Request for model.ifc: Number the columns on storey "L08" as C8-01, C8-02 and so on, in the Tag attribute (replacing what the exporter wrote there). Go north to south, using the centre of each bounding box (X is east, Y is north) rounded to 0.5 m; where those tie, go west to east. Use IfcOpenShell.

First a look at what the model holds.

```python
import ifcopenshell
import ifcopenshell.util.element
import ifcopenshell.util.placement

model = ifcopenshell.open("model.ifc")
print(model.schema)
storey = next(s for s in model.by_type("IfcBuildingStorey") if s.Name == "L08")
columns = [e for e in ifcopenshell.util.element.get_decomposition(storey) if e.is_a("IfcColumn")]
for e in sorted(columns, key=lambda e: e.id()):
    origin = ifcopenshell.util.placement.get_local_placement(e.ObjectPlacement)[:3, 3]
    print(e.id(), e.Tag, e.Name, origin.round(2) + 0.0, sep=" | ")
```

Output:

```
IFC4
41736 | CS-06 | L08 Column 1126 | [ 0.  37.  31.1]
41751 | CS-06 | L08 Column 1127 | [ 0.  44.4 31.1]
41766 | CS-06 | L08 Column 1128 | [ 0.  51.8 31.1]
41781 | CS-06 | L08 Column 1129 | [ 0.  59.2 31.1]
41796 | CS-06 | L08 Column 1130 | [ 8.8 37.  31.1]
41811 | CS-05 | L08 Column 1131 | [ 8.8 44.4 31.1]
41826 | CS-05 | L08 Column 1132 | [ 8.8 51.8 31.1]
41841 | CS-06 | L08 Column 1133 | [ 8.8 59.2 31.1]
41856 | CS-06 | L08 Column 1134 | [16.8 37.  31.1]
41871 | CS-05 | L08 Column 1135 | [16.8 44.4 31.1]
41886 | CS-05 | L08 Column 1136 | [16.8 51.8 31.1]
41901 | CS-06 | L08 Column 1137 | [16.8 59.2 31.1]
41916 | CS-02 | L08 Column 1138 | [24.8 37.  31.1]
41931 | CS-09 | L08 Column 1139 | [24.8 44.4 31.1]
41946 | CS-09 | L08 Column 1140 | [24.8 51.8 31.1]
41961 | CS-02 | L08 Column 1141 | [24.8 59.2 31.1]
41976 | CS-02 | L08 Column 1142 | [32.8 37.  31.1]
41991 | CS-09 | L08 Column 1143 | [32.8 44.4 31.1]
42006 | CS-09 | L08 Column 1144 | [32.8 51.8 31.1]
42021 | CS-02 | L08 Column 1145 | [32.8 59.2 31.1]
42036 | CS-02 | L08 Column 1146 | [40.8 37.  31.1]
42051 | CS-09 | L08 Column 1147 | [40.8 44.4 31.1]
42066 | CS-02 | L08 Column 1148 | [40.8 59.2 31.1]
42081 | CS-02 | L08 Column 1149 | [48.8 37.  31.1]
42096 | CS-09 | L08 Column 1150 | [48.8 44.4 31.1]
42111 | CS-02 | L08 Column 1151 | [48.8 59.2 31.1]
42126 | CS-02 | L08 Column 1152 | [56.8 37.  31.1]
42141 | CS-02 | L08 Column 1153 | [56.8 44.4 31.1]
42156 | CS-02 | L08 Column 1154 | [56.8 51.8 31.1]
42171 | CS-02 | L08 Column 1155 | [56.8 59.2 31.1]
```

```python
import ifcopenshell
import ifcopenshell.geom
import ifcopenshell.util.element
import ifcopenshell.util.shape

model = ifcopenshell.open("model.ifc")
settings = ifcopenshell.geom.settings()
settings.set("use-world-coords", True)


def centre(element):
    shape = ifcopenshell.geom.create_shape(settings, element)
    return ifcopenshell.util.shape.get_bbox_centroid(shape.geometry)


storey = next(s for s in model.by_type("IfcBuildingStorey") if s.Name == "L08")
columns = [e for e in ifcopenshell.util.element.get_decomposition(storey) if e.is_a("IfcColumn")]

# Insertion points can sit at a corner or the storey origin, so sort by the geometry (in metres).
centres = {e: centre(e) for e in columns}
columns.sort(key=lambda e: (-round(centres[e][1] / 0.5), centres[e][0]))

for i, e in enumerate(columns, start=1):
    number = f"C8-{i:02d}"
    e.Tag = number
    print(e.id(), number)

model.write("model_rev.ifc")
```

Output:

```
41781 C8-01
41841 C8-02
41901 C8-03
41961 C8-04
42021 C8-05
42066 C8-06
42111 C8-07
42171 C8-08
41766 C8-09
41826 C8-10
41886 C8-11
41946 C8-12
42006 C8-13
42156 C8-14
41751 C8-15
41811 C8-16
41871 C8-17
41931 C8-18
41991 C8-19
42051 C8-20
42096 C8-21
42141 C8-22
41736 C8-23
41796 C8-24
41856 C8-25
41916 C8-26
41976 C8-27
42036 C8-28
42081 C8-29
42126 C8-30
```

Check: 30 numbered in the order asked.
